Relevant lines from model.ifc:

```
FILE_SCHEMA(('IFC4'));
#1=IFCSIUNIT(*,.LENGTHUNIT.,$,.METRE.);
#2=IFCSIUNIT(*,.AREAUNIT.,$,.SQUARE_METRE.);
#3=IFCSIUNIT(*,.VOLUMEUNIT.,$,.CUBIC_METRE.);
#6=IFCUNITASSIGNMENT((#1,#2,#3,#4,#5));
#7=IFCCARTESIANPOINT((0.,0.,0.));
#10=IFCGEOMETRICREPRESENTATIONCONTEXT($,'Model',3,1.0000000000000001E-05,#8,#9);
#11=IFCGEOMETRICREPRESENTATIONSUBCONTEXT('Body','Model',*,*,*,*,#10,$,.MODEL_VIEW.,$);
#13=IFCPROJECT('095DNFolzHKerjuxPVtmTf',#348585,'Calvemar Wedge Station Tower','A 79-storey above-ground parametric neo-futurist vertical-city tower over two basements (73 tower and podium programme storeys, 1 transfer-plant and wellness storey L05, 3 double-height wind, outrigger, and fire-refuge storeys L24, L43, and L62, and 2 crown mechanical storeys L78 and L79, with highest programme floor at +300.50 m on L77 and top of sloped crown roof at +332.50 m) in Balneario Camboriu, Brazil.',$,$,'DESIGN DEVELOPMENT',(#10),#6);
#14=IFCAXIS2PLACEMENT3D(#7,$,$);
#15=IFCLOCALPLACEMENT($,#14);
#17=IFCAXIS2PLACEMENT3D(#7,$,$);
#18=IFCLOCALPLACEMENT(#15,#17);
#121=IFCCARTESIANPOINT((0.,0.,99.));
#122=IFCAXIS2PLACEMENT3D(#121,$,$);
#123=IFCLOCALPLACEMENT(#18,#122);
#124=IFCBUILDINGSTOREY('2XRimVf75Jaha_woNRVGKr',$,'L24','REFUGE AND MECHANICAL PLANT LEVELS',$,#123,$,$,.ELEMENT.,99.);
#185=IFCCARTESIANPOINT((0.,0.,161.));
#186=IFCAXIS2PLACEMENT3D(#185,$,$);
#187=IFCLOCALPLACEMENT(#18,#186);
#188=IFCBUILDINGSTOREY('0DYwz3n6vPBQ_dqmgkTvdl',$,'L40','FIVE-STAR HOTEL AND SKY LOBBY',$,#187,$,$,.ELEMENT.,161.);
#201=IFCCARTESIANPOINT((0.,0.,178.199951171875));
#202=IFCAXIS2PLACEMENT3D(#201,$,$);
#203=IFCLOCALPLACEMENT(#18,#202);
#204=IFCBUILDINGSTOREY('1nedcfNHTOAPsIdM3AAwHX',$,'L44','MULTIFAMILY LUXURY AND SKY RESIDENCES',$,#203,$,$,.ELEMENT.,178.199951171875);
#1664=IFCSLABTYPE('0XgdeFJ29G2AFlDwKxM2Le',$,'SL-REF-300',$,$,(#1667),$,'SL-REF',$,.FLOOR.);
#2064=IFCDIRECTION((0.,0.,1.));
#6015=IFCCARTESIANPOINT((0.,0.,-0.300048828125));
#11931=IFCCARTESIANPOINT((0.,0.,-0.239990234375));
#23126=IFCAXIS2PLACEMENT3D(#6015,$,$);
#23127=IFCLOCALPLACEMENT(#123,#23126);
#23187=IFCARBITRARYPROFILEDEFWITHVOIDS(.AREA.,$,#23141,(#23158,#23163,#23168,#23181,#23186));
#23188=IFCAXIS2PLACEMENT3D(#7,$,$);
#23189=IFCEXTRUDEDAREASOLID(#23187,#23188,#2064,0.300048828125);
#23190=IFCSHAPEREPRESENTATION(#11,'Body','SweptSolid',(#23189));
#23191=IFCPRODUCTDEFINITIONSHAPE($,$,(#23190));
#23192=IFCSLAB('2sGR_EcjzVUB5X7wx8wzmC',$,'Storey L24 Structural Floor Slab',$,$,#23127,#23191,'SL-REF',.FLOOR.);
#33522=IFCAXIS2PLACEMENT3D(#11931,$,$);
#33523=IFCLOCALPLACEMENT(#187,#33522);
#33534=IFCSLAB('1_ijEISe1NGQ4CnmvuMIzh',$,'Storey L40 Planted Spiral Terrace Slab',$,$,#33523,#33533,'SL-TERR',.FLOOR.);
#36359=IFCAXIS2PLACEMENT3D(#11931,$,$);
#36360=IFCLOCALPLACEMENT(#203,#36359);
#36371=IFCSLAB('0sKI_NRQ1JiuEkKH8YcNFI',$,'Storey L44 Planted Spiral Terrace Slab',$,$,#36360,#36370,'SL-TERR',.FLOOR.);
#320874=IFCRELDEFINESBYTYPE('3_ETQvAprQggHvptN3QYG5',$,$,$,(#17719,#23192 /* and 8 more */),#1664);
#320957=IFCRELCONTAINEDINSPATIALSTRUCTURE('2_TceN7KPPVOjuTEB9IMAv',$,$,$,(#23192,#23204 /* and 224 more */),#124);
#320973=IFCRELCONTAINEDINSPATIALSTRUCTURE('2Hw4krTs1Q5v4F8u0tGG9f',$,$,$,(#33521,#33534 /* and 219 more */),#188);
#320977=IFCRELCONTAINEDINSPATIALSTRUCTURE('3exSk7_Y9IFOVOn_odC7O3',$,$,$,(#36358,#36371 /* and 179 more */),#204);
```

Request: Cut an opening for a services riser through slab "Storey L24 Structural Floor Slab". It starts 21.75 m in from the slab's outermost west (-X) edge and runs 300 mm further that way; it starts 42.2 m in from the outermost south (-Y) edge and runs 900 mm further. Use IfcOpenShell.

```python
import numpy as np
import ifcopenshell
import ifcopenshell.api.feature
import ifcopenshell.api.geometry
import ifcopenshell.api.root
import ifcopenshell.geom
import ifcopenshell.util.placement
import ifcopenshell.util.representation
import ifcopenshell.util.shape
import ifcopenshell.util.unit

model = ifcopenshell.open("model.ifc")
unit_scale = ifcopenshell.util.unit.calculate_unit_scale(model)
settings = ifcopenshell.geom.settings()


def volume(element):
    """Net volume in cubic metres, openings subtracted."""
    shape = ifcopenshell.geom.create_shape(settings, element)
    return ifcopenshell.util.shape.get_volume(shape.geometry)


slab = model.by_guid("2sGR_EcjzVUB5X7wx8wzmC")
before = volume(slab)

# Extent in the slab's own axes, in metres. The edges named are its -X and -Y sides.
slab_shape = ifcopenshell.geom.create_shape(settings, slab)
vertices = ifcopenshell.util.shape.get_vertices(slab_shape.geometry)
x_min, y_min, bottom = vertices.min(axis=0)
top = vertices[:, 2].max()

opening = ifcopenshell.api.root.create_entity(model, ifc_class="IfcOpeningElement", name="Services riser opening", predefined_type="OPENING")
context = ifcopenshell.util.representation.get_context(model, "Model", "Body", "MODEL_VIEW")
width, depth = 0.3, 0.9
outline = [(0.0, 0.0), (width, 0.0), (width, depth), (0.0, depth), (0.0, 0.0)]
# Overshoot both faces by 50 mm so the cut is clean.
shape = ifcopenshell.api.geometry.add_slab_representation(
    model, context=context, depth=top - bottom + 0.1, polyline=outline
)
ifcopenshell.api.geometry.assign_representation(model, product=opening, representation=shape)

matrix = ifcopenshell.util.placement.get_local_placement(slab.ObjectPlacement)
matrix[:, 3] = matrix @ np.append(np.array([x_min + 21.75, y_min + 42.2, bottom - 0.05]) / unit_scale, 1.0)
ifcopenshell.api.geometry.edit_object_placement(model, product=opening, matrix=matrix, is_si=False)
ifcopenshell.api.feature.add_feature(model, feature=opening, element=slab)

after = volume(slab)

print(f"slab volume {before:.3f} -> {after:.3f} m3")

model.write("model_v2.ifc")
```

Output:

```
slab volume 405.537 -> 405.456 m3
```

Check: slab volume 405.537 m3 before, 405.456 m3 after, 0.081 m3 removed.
